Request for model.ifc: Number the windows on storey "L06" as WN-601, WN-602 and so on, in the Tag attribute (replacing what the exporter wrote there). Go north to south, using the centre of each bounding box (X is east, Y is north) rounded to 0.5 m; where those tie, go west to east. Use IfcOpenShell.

First a look at what the model holds.

```python
import ifcopenshell
import ifcopenshell.util.element
import ifcopenshell.util.placement

model = ifcopenshell.open("model.ifc")
print(model.schema)
storey = next(s for s in model.by_type("IfcBuildingStorey") if s.Name == "L06")
windows = [e for e in ifcopenshell.util.element.get_decomposition(storey) if e.is_a("IfcWindow")]
for e in sorted(windows, key=lambda e: e.id()):
    origin = ifcopenshell.util.placement.get_local_placement(e.ObjectPlacement)[:3, 3]
    print(e.id(), e.Tag, e.Name, origin.round(2) + 0.0, sep=" | ")
```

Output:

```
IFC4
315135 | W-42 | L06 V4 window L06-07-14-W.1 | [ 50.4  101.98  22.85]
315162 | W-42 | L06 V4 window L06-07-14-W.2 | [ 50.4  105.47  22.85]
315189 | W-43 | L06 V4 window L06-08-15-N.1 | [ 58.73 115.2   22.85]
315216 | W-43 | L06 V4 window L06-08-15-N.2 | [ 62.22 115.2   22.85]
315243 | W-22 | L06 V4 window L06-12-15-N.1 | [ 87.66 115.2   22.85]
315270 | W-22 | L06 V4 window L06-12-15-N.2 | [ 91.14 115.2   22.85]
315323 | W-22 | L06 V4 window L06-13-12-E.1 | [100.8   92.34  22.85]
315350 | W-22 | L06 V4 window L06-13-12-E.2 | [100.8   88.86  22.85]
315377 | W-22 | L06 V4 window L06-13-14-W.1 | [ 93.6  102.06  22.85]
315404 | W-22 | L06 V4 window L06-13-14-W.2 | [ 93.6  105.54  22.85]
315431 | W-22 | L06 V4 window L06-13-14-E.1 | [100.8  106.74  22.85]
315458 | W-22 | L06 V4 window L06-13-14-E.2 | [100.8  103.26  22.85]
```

```python
import ifcopenshell
import ifcopenshell.geom
import ifcopenshell.util.element
import ifcopenshell.util.shape

model = ifcopenshell.open("model.ifc")
settings = ifcopenshell.geom.settings()
settings.set("use-world-coords", True)


def centre(element):
    shape = ifcopenshell.geom.create_shape(settings, element)
    return ifcopenshell.util.shape.get_bbox_centroid(shape.geometry)


storey = next(s for s in model.by_type("IfcBuildingStorey") if s.Name == "L06")
windows = [e for e in ifcopenshell.util.element.get_decomposition(storey) if e.is_a("IfcWindow")]

# Insertion points can sit at a corner or the storey origin, so sort by the geometry (in metres).
centres = {e: centre(e) for e in windows}
windows.sort(key=lambda e: (-round(centres[e][1] / 0.5), centres[e][0]))

for i, e in enumerate(windows, start=1):
    number = f"WN-6{i:02d}"
    e.Tag = number
    print(e.id(), number)

model.write("model_updated.ifc")
```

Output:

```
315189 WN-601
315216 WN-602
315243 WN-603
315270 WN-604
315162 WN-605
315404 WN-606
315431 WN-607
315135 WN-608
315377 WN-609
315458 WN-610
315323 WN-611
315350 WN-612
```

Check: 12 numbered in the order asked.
